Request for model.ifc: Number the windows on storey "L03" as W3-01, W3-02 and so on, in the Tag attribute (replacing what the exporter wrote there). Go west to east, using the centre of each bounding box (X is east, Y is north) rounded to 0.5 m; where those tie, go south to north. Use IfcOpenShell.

First a look at what the model holds.

```python
import ifcopenshell
import ifcopenshell.util.element
import ifcopenshell.util.placement

model = ifcopenshell.open("model.ifc")
print(model.schema)
storey = next(s for s in model.by_type("IfcBuildingStorey") if s.Name == "L03")
windows = [e for e in ifcopenshell.util.element.get_decomposition(storey) if e.is_a("IfcWindow")]
for e in sorted(windows, key=lambda e: e.id()):
    origin = ifcopenshell.util.placement.get_local_placement(e.ObjectPlacement)[:3, 3]
    print(e.id(), e.Tag, e.Name, origin.round(2) + 0.0, sep=" | ")
```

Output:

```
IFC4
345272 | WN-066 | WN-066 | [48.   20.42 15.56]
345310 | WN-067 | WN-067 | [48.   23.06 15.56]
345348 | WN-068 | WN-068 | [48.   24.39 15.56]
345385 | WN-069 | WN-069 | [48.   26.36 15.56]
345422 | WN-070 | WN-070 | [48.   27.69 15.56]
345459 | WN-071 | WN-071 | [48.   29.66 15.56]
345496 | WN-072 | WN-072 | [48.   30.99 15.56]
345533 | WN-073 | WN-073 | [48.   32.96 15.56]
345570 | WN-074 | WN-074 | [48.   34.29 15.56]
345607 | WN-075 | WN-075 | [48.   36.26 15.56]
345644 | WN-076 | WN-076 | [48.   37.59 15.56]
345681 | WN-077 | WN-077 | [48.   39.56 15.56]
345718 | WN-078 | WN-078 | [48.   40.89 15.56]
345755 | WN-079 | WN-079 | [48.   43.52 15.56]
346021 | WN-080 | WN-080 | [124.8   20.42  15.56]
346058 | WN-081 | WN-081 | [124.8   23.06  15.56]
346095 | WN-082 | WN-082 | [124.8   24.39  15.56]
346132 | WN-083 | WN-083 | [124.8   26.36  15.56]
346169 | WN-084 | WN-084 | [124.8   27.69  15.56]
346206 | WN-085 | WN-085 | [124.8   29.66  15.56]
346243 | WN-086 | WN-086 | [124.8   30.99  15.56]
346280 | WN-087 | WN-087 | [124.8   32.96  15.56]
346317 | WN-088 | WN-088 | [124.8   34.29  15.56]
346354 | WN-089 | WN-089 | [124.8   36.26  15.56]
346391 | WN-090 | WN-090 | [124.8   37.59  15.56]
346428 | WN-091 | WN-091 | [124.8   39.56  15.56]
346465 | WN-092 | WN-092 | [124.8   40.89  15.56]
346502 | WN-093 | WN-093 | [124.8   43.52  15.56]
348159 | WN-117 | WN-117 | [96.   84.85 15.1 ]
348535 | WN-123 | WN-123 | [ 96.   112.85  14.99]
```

```python
import ifcopenshell
import ifcopenshell.geom
import ifcopenshell.util.element
import ifcopenshell.util.shape

model = ifcopenshell.open("model.ifc")
settings = ifcopenshell.geom.settings()
settings.set("use-world-coords", True)


def centre(element):
    shape = ifcopenshell.geom.create_shape(settings, element)
    return ifcopenshell.util.shape.get_bbox_centroid(shape.geometry)


storey = next(s for s in model.by_type("IfcBuildingStorey") if s.Name == "L03")
windows = [e for e in ifcopenshell.util.element.get_decomposition(storey) if e.is_a("IfcWindow")]

# Insertion points can sit at a corner or the storey origin, so sort by the geometry (in metres).
centres = {e: centre(e) for e in windows}
windows.sort(key=lambda e: (round(centres[e][0] / 0.5), centres[e][1]))

for i, e in enumerate(windows, start=1):
    number = f"W3-{i:02d}"
    e.Tag = number
    print(e.id(), number)

model.write("model_edited.ifc")
```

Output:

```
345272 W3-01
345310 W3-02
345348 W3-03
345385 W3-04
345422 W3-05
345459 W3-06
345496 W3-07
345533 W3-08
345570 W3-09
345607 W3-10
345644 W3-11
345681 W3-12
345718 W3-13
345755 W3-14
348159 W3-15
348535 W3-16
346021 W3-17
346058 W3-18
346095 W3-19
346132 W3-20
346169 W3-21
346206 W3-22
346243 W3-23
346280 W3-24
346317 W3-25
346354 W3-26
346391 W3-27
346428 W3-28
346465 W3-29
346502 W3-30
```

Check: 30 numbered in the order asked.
